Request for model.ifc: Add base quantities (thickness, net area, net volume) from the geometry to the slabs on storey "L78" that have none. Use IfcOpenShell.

First a look at what the model holds.

```python
import ifcopenshell
import ifcopenshell.util.element
import ifcopenshell.util.unit

model = ifcopenshell.open("model.ifc")
print(model.schema)
for unit_type in ("LENGTHUNIT", "AREAUNIT", "VOLUMEUNIT"):
    print(unit_type, ifcopenshell.util.unit.calculate_unit_scale(model, unit_type))
storey = next(s for s in model.by_type("IfcBuildingStorey") if s.Name == "L78")
slabs = [e for e in ifcopenshell.util.element.get_decomposition(storey) if e.is_a("IfcSlab")]
for e in sorted(slabs, key=lambda e: e.id()):
    print(e.id(), e.is_a(), e.Name, list(ifcopenshell.util.element.get_psets(e, qtos_only=True)), sep=" | ")
```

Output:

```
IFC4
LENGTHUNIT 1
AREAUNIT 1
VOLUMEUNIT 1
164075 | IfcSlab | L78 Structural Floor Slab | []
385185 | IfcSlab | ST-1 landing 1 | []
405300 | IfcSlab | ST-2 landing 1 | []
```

```python
import ifcopenshell
import ifcopenshell.api.pset
import ifcopenshell.geom
import ifcopenshell.util.element
import ifcopenshell.util.shape
import ifcopenshell.util.unit

model = ifcopenshell.open("model.ifc")
unit_scale = ifcopenshell.util.unit.calculate_unit_scale(model)
area_scale = ifcopenshell.util.unit.calculate_unit_scale(model, "AREAUNIT")
volume_scale = ifcopenshell.util.unit.calculate_unit_scale(model, "VOLUMEUNIT")
settings = ifcopenshell.geom.settings()

storey = next(s for s in model.by_type("IfcBuildingStorey") if s.Name == "L78")
slabs = [e for e in ifcopenshell.util.element.get_decomposition(storey) if e.is_a("IfcSlab")]

for e in sorted(slabs, key=lambda e: e.id()):
    if ifcopenshell.util.element.get_psets(e, qtos_only=True, should_inherit=False):
        continue
    # Geometry comes back in metres, in the element's own axes.
    shape = ifcopenshell.geom.create_shape(settings, e)
    values = {
        "Width": ifcopenshell.util.shape.get_z(shape.geometry) / unit_scale,
        "NetArea": ifcopenshell.util.shape.get_footprint_area(shape.geometry) / area_scale,
        "NetVolume": ifcopenshell.util.shape.get_volume(shape.geometry) / volume_scale,
    }
    qto = ifcopenshell.api.pset.add_qto(model, product=e, name="Qto_SlabBaseQuantities")
    ifcopenshell.api.pset.edit_qto(model, qto=qto, properties=values)
    print(e.id(), {k: round(v, 3) for k, v in values.items()})

model.write("model_rev.ifc")
```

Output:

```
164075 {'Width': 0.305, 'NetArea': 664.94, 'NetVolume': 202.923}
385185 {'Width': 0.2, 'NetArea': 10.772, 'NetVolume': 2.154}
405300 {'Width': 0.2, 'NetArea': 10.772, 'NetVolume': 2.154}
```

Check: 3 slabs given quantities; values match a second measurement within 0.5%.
